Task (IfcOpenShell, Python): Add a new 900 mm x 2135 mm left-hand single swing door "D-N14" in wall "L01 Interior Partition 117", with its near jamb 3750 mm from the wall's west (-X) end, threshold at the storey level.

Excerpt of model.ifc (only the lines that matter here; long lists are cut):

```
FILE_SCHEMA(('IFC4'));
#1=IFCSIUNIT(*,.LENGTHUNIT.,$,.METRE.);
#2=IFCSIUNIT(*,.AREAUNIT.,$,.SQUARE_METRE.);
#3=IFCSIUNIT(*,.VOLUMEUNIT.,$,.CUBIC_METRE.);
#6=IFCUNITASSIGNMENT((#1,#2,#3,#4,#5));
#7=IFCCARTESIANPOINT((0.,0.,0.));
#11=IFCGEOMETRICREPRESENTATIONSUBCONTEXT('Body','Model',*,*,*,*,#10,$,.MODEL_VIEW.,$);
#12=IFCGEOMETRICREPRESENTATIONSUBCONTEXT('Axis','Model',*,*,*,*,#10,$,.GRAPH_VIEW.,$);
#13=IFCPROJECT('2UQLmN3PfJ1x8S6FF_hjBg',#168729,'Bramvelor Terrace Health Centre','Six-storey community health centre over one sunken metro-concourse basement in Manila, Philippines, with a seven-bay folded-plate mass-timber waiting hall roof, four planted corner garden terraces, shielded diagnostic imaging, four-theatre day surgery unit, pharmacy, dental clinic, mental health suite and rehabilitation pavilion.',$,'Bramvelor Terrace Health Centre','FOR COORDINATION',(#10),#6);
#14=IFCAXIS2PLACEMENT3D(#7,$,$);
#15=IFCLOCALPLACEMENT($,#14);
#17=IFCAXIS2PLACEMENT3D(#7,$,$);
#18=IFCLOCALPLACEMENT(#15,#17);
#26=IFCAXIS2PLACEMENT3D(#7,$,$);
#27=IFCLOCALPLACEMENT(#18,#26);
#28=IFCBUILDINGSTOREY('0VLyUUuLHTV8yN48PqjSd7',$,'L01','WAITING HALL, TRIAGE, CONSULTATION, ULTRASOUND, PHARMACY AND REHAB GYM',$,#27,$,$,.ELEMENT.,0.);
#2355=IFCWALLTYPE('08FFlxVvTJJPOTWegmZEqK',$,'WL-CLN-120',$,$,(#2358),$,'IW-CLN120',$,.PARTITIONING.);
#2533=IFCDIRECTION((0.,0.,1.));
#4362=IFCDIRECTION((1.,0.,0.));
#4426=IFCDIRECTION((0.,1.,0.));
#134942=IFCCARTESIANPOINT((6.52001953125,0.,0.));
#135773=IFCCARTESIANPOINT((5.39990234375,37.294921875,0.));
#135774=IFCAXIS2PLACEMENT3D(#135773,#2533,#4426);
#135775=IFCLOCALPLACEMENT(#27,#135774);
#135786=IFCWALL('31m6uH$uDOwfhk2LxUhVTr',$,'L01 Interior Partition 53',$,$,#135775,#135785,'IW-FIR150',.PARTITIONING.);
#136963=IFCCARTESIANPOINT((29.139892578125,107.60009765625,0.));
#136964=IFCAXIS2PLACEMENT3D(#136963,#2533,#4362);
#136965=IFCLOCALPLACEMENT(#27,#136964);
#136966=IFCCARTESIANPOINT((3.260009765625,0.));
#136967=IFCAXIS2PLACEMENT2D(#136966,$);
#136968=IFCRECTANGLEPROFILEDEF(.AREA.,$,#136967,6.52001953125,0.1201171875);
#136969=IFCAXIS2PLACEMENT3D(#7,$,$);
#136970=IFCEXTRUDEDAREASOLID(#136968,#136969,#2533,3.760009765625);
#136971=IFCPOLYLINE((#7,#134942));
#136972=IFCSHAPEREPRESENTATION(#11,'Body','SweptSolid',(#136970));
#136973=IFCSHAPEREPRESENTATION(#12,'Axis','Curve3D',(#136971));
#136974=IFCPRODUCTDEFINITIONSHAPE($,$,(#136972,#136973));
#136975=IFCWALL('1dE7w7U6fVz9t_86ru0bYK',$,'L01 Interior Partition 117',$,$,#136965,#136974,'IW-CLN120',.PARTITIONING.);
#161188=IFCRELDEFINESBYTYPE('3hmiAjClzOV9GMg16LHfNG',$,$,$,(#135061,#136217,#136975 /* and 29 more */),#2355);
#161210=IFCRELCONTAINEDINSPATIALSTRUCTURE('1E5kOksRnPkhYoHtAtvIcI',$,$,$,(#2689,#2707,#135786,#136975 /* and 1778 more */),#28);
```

```python
import numpy as np
import ifcopenshell
import ifcopenshell.api.feature
import ifcopenshell.api.geometry
import ifcopenshell.api.root
import ifcopenshell.api.spatial
import ifcopenshell.geom
import ifcopenshell.util.element
import ifcopenshell.util.placement
import ifcopenshell.util.representation
import ifcopenshell.util.shape
import ifcopenshell.util.unit

model = ifcopenshell.open("model.ifc")
unit_scale = ifcopenshell.util.unit.calculate_unit_scale(model)
settings = ifcopenshell.geom.settings()


def volume(element):
    """Net volume in cubic metres, openings subtracted."""
    shape = ifcopenshell.geom.create_shape(settings, element)
    return ifcopenshell.util.shape.get_volume(shape.geometry)


wall = model.by_id(136975)
storey = ifcopenshell.util.element.get_container(wall, ifc_class="IfcBuildingStorey")
context = ifcopenshell.util.representation.get_context(model, "Model", "Body", "MODEL_VIEW")
before = volume(wall)

width, height, from_end, sill = 0.9, 2.135, 3.75, 0.0  # metres

# The wall runs along its own X axis, and the end named is its -X end.
wall_shape = ifcopenshell.geom.create_shape(settings, wall)
x, y, z = ifcopenshell.util.shape.get_vertices(wall_shape.geometry).T
start = x.min() + from_end
face, thickness = float(y.min()), float(y.max() - y.min())
wall_matrix = ifcopenshell.util.placement.get_local_placement(wall.ObjectPlacement)
level = ifcopenshell.util.placement.get_local_placement(storey.ObjectPlacement)[2, 3]


def in_wall(x, y):
    """Placement at x, y metres in the wall's axes, at sill height."""
    matrix = wall_matrix.copy()
    matrix[:, 3] = wall_matrix @ np.array([x / unit_scale, y / unit_scale, 0.0, 1.0])
    matrix[2, 3] = level + sill / unit_scale
    return matrix


# Opening: a box that overshoots both wall faces by 50 mm.
opening = ifcopenshell.api.root.create_entity(model, ifc_class="IfcOpeningElement", predefined_type="OPENING")
box = ifcopenshell.api.geometry.add_wall_representation(
    model, context=context, length=width, height=height, thickness=thickness + 0.1
)
ifcopenshell.api.geometry.assign_representation(model, product=opening, representation=box)
ifcopenshell.api.geometry.edit_object_placement(model, product=opening, matrix=in_wall(start, face - 0.05), is_si=False)
ifcopenshell.api.feature.add_feature(model, feature=opening, element=wall)

door = ifcopenshell.api.root.create_entity(model, ifc_class="IfcDoor", name="D-N14", predefined_type="DOOR")
door.OverallWidth, door.OverallHeight = width / unit_scale, height / unit_scale
door.OperationType = "SINGLE_SWING_LEFT"
body = ifcopenshell.api.geometry.add_door_representation(
    model,
    context=context,
    overall_width=door.OverallWidth,
    overall_height=door.OverallHeight,
    operation_type="SINGLE_SWING_LEFT",
    lining_properties={"LiningDepth": thickness / unit_scale, "ThresholdDepth": thickness / unit_scale},
)
ifcopenshell.api.geometry.assign_representation(model, product=door, representation=body)
ifcopenshell.api.spatial.assign_container(model, products=[door], relating_structure=storey)
ifcopenshell.api.feature.add_filling(model, opening=opening, element=door)

# The lining spans the wall, so the door starts at the wall face.
ifcopenshell.api.geometry.edit_object_placement(model, product=door, matrix=in_wall(start, face), is_si=False)

after = volume(wall)

print(f"wall volume {before:.3f} -> {after:.3f} m3")

model.write("model_edited.ifc")
```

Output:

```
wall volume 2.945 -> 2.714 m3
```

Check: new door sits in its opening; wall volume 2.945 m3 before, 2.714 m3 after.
